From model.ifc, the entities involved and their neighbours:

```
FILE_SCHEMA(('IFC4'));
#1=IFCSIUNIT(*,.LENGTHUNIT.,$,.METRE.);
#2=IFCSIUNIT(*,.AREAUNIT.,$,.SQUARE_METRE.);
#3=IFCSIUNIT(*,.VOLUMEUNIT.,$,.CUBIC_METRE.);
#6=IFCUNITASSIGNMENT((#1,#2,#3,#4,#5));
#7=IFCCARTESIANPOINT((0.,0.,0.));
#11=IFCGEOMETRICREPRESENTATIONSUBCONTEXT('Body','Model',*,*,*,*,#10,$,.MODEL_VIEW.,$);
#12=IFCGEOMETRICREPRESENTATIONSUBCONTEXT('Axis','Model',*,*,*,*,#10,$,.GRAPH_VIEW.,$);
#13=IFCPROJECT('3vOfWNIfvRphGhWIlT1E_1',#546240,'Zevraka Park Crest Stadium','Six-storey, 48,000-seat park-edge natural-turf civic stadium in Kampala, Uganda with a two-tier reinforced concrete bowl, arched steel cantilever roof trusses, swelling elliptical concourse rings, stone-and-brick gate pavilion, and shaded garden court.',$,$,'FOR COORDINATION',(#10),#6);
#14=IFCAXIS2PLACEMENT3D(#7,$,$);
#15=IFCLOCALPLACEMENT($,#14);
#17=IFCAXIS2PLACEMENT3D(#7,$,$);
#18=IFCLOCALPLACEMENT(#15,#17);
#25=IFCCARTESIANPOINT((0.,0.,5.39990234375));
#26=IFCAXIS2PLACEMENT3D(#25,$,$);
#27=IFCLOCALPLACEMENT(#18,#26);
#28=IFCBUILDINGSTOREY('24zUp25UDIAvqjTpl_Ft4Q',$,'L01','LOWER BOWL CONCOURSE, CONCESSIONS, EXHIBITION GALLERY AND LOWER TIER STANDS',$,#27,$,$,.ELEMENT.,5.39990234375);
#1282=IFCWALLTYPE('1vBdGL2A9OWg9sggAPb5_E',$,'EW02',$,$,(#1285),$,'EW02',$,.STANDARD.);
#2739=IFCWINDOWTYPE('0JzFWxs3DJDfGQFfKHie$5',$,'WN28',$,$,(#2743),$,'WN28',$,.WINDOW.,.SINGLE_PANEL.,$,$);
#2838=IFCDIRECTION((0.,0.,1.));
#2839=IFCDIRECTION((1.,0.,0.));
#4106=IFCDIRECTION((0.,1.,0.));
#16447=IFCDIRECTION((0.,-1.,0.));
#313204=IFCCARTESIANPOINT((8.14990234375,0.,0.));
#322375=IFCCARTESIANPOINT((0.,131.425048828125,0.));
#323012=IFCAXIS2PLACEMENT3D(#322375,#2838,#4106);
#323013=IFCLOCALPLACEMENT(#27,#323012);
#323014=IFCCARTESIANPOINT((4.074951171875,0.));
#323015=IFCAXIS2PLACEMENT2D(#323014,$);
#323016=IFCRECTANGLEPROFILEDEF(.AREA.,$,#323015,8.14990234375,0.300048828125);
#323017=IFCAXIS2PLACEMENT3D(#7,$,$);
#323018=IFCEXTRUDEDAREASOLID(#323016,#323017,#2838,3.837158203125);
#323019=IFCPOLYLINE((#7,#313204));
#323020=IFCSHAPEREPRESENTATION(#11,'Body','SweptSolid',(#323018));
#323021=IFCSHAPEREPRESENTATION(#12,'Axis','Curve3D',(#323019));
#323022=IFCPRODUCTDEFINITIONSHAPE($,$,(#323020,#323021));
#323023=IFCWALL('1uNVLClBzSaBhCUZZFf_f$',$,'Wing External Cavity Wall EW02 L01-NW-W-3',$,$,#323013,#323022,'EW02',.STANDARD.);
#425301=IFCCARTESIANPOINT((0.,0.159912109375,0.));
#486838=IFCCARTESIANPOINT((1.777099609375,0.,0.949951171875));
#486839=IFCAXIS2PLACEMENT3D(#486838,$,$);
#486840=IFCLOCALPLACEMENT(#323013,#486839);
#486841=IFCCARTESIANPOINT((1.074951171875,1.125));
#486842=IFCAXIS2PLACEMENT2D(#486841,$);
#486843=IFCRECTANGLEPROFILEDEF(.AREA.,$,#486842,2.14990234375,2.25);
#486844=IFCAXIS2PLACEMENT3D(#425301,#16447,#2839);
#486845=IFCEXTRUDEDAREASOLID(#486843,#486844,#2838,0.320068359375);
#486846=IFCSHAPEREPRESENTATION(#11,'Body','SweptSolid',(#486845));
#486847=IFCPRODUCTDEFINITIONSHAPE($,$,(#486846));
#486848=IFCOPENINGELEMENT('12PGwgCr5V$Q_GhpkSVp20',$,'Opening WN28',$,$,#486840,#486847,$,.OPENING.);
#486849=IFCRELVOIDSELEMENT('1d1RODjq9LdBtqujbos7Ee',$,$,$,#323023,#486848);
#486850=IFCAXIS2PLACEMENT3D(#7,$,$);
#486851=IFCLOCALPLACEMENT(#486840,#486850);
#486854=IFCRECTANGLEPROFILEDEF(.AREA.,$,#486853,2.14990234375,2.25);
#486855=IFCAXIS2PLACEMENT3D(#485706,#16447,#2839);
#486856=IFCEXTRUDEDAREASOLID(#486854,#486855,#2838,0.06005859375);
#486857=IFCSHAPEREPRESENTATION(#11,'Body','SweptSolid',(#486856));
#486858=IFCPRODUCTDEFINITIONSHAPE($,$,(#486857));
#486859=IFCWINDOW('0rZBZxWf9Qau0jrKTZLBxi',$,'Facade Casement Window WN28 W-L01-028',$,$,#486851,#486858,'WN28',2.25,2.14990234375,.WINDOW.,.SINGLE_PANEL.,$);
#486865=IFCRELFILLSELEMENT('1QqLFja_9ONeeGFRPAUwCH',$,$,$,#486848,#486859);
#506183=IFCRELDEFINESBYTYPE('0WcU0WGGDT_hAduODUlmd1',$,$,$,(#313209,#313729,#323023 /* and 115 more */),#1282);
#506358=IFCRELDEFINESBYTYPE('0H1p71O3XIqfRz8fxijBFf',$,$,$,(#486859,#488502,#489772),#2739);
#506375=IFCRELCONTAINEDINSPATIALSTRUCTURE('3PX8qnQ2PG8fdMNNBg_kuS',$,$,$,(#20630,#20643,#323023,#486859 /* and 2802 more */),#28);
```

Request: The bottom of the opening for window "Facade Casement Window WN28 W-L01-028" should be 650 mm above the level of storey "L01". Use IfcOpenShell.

```python
import numpy as np
import ifcopenshell
import ifcopenshell.api.geometry
import ifcopenshell.geom
import ifcopenshell.util.element
import ifcopenshell.util.placement
import ifcopenshell.util.shape
import ifcopenshell.util.unit

model = ifcopenshell.open("model.ifc")
unit_scale = ifcopenshell.util.unit.calculate_unit_scale(model)

window = model.by_guid("0rZBZxWf9Qau0jrKTZLBxi")
opening = window.FillsVoids[0].RelatingOpeningElement
storey = ifcopenshell.util.element.get_container(window, ifc_class="IfcBuildingStorey")
level = ifcopenshell.util.placement.get_local_placement(storey.ObjectPlacement)[2, 3]

# The opening's origin need not be at the sill, so measure its lowest point.
shape = ifcopenshell.geom.create_shape(ifcopenshell.geom.settings(), opening)
bottom = ifcopenshell.util.shape.get_shape_bottom_elevation(shape, shape.geometry) / unit_scale
dz = level + 0.65 - bottom

shift = np.array([0.0, 0.0, dz])
# The window is placed relative to its opening, so it follows when the opening moves.
matrix = ifcopenshell.util.placement.get_local_placement(opening.ObjectPlacement)
matrix[:3, 3] += shift
ifcopenshell.api.geometry.edit_object_placement(
    model, product=opening, matrix=matrix, is_si=False, should_transform_children=True
)

print(f"moved by {dz * unit_scale:+.3f} m")

model.write("model_rev.ifc")
```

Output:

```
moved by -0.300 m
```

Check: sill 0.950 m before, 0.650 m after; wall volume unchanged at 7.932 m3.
